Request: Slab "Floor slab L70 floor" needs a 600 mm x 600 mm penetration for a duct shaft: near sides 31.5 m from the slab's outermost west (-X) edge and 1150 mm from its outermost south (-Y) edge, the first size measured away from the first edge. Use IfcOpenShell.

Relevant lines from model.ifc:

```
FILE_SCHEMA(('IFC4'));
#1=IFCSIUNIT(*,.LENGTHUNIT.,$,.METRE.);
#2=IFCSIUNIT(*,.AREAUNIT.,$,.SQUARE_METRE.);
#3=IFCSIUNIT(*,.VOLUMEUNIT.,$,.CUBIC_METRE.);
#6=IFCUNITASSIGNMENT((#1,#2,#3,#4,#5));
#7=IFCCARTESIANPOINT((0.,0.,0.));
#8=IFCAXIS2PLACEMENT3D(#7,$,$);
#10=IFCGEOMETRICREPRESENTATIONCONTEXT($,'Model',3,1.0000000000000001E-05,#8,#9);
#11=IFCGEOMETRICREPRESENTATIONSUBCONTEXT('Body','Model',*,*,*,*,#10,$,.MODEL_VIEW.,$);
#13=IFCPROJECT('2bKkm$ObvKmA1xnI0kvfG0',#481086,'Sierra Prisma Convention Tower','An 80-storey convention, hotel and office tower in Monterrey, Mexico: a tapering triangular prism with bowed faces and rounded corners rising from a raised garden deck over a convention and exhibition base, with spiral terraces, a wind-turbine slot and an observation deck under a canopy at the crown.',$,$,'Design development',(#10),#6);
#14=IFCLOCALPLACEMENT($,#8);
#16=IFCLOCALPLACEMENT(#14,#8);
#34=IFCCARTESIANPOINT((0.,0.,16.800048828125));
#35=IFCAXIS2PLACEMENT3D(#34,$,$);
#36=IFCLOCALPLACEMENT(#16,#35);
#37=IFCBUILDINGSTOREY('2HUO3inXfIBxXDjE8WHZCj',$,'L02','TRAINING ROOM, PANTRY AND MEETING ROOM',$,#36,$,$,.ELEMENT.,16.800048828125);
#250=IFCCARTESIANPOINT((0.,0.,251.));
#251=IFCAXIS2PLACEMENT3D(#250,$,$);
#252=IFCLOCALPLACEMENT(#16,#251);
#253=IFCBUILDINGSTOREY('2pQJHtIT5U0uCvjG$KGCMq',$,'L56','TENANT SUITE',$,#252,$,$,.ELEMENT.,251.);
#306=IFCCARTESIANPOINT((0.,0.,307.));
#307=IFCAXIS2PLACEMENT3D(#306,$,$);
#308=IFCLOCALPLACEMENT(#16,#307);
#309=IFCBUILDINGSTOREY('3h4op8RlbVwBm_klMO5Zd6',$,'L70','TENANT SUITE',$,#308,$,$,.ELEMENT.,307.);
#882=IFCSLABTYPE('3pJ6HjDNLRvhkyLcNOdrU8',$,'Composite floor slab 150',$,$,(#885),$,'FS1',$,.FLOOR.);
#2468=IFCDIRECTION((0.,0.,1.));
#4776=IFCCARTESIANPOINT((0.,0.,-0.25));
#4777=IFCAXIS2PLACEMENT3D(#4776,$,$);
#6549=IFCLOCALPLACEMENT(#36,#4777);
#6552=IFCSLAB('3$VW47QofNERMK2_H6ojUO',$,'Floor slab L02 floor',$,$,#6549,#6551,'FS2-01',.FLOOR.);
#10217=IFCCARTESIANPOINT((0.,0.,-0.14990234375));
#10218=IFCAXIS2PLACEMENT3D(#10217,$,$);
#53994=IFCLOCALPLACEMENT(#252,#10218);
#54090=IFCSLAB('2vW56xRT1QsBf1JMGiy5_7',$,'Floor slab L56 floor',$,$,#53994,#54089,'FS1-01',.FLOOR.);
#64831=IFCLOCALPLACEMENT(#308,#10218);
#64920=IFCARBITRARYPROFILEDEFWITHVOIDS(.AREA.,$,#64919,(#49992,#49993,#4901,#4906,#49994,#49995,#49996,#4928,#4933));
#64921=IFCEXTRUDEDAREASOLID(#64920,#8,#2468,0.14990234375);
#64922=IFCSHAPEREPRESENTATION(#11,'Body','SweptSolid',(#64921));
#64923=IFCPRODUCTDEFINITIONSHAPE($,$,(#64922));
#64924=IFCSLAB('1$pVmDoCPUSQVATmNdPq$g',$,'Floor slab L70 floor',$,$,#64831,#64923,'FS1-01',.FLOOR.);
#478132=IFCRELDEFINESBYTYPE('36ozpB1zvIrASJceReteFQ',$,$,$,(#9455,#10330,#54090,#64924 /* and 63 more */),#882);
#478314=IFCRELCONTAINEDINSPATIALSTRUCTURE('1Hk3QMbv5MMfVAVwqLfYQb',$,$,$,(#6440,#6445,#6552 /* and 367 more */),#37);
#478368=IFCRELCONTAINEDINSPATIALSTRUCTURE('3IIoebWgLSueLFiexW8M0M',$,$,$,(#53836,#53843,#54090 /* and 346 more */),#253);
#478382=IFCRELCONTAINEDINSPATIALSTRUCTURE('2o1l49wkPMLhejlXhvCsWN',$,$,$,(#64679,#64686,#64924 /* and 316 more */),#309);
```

```python
import numpy as np
import ifcopenshell
import ifcopenshell.api.feature
import ifcopenshell.api.geometry
import ifcopenshell.api.root
import ifcopenshell.geom
import ifcopenshell.util.placement
import ifcopenshell.util.representation
import ifcopenshell.util.shape
import ifcopenshell.util.unit

model = ifcopenshell.open("model.ifc")
unit_scale = ifcopenshell.util.unit.calculate_unit_scale(model)
settings = ifcopenshell.geom.settings()


def volume(element):
    """Net volume in cubic metres, openings subtracted."""
    shape = ifcopenshell.geom.create_shape(settings, element)
    return ifcopenshell.util.shape.get_volume(shape.geometry)


slab = model.by_guid("1$pVmDoCPUSQVATmNdPq$g")
before = volume(slab)

# Extent in the slab's own axes, in metres. The edges named are its -X and -Y sides.
slab_shape = ifcopenshell.geom.create_shape(settings, slab)
vertices = ifcopenshell.util.shape.get_vertices(slab_shape.geometry)
x_min, y_min, bottom = vertices.min(axis=0)
top = vertices[:, 2].max()

opening = ifcopenshell.api.root.create_entity(model, ifc_class="IfcOpeningElement", name="Duct shaft opening", predefined_type="OPENING")
context = ifcopenshell.util.representation.get_context(model, "Model", "Body", "MODEL_VIEW")
width, depth = 0.6, 0.6
outline = [(0.0, 0.0), (width, 0.0), (width, depth), (0.0, depth), (0.0, 0.0)]
# Overshoot both faces by 50 mm so the cut is clean.
shape = ifcopenshell.api.geometry.add_slab_representation(
    model, context=context, depth=top - bottom + 0.1, polyline=outline
)
ifcopenshell.api.geometry.assign_representation(model, product=opening, representation=shape)

matrix = ifcopenshell.util.placement.get_local_placement(slab.ObjectPlacement)
matrix[:, 3] = matrix @ np.append(np.array([x_min + 31.5, y_min + 1.15, bottom - 0.05]) / unit_scale, 1.0)
ifcopenshell.api.geometry.edit_object_placement(model, product=opening, matrix=matrix, is_si=False)
ifcopenshell.api.feature.add_feature(model, feature=opening, element=slab)

after = volume(slab)

print(f"slab volume {before:.3f} -> {after:.3f} m3")

model.write("model_updated.ifc")
```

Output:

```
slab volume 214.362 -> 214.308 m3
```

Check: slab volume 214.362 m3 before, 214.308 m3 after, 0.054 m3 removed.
